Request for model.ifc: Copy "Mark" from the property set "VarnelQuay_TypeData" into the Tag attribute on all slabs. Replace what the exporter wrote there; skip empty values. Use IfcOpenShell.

First a look at what the model holds.

```python
import ifcopenshell
import ifcopenshell.util.element

model = ifcopenshell.open("model.ifc")
print(model.schema)
slabs = model.by_type("IfcSlab")
print(len(slabs), "slabs")
for e in slabs[:8]:
    source = ifcopenshell.util.element.get_pset(e, "VarnelQuay_TypeData", "Mark")
    target = e.Tag
    print(e.id(), repr(source), repr(target), sep=" | ")
```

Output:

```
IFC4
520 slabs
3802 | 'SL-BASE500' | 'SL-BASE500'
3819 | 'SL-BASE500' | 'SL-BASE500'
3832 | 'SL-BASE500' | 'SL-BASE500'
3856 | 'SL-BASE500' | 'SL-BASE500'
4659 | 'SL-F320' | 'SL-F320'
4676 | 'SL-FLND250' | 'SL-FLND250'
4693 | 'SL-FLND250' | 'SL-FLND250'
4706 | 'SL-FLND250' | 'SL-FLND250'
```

```python
import ifcopenshell
import ifcopenshell.util.element

model = ifcopenshell.open("model.ifc")

count = 0
for e in model.by_type("IfcSlab"):
    value = ifcopenshell.util.element.get_pset(e, "VarnelQuay_TypeData", "Mark")
    current = e.Tag
    if not value or not value.strip() or current == value:
        continue
    e.Tag = value
    count += 1

print(count, "slabs updated")

model.write("model_updated.ifc")
```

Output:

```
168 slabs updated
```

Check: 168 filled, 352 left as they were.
